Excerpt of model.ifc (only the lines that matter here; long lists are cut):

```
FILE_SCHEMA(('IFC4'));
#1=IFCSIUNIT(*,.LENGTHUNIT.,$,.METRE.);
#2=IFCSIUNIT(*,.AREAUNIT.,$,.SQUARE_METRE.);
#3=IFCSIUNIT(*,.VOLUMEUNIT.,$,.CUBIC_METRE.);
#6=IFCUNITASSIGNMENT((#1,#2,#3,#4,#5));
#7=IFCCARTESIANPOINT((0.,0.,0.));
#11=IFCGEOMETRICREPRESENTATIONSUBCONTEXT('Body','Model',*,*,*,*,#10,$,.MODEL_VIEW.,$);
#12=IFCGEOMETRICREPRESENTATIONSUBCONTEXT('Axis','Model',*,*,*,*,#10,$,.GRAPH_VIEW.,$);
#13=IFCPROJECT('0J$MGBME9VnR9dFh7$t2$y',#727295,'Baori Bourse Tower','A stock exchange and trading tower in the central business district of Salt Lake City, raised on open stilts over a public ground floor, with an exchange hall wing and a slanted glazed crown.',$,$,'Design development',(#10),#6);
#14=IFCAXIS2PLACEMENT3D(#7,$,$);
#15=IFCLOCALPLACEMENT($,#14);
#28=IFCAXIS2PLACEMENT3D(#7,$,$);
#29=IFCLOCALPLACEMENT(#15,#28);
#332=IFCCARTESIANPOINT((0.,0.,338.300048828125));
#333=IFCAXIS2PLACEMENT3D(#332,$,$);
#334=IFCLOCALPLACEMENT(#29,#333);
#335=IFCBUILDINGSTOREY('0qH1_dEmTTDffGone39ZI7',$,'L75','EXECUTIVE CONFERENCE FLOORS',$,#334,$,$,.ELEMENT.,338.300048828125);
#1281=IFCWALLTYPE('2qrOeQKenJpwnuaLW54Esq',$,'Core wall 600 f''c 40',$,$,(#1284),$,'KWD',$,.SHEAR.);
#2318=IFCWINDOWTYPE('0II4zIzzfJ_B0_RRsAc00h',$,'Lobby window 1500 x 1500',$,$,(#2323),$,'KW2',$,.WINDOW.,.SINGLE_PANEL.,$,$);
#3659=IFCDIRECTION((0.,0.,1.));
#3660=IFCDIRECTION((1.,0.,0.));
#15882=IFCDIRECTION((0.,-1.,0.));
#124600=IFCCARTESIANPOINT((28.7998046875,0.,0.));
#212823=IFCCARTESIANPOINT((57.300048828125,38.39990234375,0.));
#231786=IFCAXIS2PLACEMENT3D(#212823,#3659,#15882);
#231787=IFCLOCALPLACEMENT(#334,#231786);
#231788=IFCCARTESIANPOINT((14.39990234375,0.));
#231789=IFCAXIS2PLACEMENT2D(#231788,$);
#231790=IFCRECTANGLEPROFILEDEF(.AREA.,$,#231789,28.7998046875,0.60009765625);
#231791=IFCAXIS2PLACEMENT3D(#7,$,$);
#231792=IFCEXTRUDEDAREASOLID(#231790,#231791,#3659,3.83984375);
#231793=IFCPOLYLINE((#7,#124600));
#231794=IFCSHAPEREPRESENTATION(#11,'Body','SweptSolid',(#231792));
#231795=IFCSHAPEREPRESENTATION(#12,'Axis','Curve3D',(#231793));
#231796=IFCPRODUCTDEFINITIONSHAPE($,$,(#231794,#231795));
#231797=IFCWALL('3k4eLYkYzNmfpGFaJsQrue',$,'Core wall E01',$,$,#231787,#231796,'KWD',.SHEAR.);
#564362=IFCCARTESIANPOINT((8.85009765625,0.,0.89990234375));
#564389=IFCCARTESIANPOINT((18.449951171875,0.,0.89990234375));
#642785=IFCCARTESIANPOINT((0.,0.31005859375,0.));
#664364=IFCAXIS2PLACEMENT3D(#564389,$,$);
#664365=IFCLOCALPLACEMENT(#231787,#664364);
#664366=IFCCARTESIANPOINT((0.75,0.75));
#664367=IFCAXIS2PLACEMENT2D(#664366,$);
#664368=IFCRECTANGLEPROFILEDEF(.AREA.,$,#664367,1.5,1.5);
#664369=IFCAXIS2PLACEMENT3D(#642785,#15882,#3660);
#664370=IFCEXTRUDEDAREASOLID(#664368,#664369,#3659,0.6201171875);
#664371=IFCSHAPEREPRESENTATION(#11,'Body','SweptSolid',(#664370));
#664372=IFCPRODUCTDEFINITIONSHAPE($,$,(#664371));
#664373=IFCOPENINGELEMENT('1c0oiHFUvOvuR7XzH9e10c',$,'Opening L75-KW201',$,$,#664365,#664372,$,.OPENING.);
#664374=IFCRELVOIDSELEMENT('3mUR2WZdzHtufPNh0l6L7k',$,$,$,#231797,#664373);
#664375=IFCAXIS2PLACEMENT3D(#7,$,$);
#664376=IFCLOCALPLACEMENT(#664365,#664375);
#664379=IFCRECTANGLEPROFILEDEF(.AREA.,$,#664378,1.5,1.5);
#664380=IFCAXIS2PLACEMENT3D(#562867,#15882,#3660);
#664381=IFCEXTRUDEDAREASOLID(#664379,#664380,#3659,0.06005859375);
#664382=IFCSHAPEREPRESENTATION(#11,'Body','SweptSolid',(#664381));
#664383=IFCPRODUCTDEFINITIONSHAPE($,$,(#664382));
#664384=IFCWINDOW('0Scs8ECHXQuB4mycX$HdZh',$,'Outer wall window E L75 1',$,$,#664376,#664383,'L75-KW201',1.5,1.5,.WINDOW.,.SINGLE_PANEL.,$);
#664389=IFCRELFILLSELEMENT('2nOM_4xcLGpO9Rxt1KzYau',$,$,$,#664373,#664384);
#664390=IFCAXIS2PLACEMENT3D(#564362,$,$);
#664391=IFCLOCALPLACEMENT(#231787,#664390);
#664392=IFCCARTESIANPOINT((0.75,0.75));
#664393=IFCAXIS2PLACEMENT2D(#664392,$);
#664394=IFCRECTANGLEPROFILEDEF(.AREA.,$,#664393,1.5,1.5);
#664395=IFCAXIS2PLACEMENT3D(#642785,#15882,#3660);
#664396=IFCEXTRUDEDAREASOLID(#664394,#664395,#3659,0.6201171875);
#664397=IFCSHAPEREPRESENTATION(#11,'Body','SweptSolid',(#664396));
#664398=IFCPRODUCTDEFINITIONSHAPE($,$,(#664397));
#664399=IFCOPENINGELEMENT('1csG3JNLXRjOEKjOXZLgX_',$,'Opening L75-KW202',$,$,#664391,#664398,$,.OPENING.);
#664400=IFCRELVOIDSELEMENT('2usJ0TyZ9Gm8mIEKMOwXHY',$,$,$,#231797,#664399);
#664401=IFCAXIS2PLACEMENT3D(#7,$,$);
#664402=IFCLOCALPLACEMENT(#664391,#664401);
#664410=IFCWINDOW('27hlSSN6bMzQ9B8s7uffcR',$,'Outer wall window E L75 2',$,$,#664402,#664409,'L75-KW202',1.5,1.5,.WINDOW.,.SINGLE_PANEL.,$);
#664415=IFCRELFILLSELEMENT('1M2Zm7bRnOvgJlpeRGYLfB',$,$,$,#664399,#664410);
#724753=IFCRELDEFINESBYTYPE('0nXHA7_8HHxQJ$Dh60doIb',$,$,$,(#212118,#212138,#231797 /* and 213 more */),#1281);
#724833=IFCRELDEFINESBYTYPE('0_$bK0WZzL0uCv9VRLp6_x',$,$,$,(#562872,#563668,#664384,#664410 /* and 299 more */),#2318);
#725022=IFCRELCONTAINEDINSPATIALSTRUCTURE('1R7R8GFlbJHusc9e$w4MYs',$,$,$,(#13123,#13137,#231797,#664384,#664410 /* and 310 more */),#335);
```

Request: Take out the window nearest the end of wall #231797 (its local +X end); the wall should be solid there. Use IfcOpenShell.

```python
import ifcopenshell
import ifcopenshell.api.feature
import ifcopenshell.api.root
import ifcopenshell.geom
import ifcopenshell.util.shape

model = ifcopenshell.open("model.ifc")
settings = ifcopenshell.geom.settings()


def volume(element):
    """Net volume in cubic metres, openings subtracted."""
    shape = ifcopenshell.geom.create_shape(settings, element)
    return ifcopenshell.util.shape.get_volume(shape.geometry)


window = model.by_guid("0Scs8ECHXQuB4mycX$HdZh")
opening = window.FillsVoids[0].RelatingOpeningElement
wall = opening.VoidsElements[0].RelatingBuildingElement
before = volume(wall)

ifcopenshell.api.root.remove_product(model, product=window)
ifcopenshell.api.feature.remove_feature(model, feature=opening)

after = volume(wall)

print(f"wall volume {before:.3f} -> {after:.3f} m3")

model.write("model_updated.ifc")
```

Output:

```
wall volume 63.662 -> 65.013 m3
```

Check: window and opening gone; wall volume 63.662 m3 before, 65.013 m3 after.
